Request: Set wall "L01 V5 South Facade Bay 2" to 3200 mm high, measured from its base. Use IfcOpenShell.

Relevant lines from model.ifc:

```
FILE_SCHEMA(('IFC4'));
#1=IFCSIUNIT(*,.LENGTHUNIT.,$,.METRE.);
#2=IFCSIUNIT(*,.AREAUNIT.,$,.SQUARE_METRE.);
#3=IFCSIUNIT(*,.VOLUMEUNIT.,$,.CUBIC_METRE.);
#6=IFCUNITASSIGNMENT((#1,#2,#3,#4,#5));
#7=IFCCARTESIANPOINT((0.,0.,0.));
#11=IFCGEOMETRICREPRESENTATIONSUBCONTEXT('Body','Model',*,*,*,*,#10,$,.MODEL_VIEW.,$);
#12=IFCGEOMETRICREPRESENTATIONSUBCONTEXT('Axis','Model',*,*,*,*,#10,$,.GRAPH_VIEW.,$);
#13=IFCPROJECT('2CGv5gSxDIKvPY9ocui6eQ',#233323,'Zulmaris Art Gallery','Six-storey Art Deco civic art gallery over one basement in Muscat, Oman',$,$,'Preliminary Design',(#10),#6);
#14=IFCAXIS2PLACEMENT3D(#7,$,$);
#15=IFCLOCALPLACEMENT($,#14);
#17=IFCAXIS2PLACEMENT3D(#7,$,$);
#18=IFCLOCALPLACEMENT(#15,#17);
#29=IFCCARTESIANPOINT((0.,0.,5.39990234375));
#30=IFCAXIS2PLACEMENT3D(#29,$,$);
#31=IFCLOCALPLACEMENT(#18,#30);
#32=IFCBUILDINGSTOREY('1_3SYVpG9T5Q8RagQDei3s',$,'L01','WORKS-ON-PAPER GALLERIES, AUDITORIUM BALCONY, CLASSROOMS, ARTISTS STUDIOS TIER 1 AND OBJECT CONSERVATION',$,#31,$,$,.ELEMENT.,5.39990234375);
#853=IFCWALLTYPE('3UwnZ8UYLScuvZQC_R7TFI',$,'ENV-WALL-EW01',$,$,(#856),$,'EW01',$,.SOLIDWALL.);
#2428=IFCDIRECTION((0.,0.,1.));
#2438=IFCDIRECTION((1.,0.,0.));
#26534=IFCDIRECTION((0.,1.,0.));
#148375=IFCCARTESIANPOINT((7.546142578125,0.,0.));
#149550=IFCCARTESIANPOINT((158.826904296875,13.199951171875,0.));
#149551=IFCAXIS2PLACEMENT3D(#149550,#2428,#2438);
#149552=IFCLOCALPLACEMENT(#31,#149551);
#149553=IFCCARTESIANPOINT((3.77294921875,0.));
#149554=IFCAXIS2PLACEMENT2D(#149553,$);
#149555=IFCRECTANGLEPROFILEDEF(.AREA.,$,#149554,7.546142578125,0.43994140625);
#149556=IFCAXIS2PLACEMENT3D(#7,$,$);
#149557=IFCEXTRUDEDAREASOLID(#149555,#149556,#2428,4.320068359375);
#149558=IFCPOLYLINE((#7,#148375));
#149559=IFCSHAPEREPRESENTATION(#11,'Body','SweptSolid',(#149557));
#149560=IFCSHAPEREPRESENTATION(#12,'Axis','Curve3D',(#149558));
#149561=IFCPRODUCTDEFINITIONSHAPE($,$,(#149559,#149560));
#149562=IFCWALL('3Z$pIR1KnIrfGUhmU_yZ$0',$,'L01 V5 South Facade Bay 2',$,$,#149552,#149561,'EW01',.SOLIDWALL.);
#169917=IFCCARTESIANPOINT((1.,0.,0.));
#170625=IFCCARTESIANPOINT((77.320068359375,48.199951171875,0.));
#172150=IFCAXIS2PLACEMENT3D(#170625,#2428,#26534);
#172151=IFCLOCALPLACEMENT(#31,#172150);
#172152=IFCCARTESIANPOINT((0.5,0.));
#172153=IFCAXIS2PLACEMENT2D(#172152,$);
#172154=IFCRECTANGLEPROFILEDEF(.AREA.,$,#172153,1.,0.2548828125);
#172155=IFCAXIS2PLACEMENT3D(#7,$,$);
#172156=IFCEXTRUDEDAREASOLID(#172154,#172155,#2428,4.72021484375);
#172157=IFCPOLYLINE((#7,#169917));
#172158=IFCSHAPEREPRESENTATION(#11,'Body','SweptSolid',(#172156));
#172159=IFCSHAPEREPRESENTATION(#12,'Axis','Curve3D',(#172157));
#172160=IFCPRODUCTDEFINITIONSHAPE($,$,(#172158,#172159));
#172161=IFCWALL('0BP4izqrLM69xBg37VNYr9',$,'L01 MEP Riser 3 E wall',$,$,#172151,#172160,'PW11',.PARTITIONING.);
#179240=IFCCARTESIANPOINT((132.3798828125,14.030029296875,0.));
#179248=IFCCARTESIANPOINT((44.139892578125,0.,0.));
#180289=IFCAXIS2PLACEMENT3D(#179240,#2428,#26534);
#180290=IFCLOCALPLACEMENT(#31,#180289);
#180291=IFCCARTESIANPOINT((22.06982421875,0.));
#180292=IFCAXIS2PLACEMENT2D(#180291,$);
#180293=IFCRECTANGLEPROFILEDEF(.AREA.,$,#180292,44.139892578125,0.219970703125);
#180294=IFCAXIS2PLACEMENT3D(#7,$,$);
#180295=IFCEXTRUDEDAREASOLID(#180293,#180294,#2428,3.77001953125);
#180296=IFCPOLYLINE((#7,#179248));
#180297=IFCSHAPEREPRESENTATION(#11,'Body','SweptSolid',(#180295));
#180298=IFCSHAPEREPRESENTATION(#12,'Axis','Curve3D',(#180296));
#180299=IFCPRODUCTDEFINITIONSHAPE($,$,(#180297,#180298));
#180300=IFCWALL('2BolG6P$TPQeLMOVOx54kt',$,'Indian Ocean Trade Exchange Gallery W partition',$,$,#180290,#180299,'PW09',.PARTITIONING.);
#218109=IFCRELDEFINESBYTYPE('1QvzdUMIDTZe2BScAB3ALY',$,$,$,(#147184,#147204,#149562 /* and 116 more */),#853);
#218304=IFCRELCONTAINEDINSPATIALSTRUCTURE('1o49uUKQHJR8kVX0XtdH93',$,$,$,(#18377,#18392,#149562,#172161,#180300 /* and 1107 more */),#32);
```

```python
import ifcopenshell
import ifcopenshell.geom
import ifcopenshell.util.representation
import ifcopenshell.util.shape
import ifcopenshell.util.unit

model = ifcopenshell.open("model.ifc")
unit_scale = ifcopenshell.util.unit.calculate_unit_scale(model)
settings = ifcopenshell.geom.settings()


def volume(element):
    """Net volume in cubic metres, openings subtracted."""
    shape = ifcopenshell.geom.create_shape(settings, element)
    return ifcopenshell.util.shape.get_volume(shape.geometry)


wall = model.by_id(149562)
before = volume(wall)

body = ifcopenshell.util.representation.get_representation(wall, "Model", "Body")
solid = body.Items[0]
old_height = solid.Depth
solid.Depth = 3.2 / unit_scale
after = volume(wall)

print(f"height {old_height:g} -> {solid.Depth:g}, volume {before:.3f} -> {after:.3f} m3")

model.write("model_updated.ifc")
```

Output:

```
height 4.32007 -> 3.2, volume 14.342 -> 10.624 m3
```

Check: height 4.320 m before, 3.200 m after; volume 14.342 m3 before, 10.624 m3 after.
